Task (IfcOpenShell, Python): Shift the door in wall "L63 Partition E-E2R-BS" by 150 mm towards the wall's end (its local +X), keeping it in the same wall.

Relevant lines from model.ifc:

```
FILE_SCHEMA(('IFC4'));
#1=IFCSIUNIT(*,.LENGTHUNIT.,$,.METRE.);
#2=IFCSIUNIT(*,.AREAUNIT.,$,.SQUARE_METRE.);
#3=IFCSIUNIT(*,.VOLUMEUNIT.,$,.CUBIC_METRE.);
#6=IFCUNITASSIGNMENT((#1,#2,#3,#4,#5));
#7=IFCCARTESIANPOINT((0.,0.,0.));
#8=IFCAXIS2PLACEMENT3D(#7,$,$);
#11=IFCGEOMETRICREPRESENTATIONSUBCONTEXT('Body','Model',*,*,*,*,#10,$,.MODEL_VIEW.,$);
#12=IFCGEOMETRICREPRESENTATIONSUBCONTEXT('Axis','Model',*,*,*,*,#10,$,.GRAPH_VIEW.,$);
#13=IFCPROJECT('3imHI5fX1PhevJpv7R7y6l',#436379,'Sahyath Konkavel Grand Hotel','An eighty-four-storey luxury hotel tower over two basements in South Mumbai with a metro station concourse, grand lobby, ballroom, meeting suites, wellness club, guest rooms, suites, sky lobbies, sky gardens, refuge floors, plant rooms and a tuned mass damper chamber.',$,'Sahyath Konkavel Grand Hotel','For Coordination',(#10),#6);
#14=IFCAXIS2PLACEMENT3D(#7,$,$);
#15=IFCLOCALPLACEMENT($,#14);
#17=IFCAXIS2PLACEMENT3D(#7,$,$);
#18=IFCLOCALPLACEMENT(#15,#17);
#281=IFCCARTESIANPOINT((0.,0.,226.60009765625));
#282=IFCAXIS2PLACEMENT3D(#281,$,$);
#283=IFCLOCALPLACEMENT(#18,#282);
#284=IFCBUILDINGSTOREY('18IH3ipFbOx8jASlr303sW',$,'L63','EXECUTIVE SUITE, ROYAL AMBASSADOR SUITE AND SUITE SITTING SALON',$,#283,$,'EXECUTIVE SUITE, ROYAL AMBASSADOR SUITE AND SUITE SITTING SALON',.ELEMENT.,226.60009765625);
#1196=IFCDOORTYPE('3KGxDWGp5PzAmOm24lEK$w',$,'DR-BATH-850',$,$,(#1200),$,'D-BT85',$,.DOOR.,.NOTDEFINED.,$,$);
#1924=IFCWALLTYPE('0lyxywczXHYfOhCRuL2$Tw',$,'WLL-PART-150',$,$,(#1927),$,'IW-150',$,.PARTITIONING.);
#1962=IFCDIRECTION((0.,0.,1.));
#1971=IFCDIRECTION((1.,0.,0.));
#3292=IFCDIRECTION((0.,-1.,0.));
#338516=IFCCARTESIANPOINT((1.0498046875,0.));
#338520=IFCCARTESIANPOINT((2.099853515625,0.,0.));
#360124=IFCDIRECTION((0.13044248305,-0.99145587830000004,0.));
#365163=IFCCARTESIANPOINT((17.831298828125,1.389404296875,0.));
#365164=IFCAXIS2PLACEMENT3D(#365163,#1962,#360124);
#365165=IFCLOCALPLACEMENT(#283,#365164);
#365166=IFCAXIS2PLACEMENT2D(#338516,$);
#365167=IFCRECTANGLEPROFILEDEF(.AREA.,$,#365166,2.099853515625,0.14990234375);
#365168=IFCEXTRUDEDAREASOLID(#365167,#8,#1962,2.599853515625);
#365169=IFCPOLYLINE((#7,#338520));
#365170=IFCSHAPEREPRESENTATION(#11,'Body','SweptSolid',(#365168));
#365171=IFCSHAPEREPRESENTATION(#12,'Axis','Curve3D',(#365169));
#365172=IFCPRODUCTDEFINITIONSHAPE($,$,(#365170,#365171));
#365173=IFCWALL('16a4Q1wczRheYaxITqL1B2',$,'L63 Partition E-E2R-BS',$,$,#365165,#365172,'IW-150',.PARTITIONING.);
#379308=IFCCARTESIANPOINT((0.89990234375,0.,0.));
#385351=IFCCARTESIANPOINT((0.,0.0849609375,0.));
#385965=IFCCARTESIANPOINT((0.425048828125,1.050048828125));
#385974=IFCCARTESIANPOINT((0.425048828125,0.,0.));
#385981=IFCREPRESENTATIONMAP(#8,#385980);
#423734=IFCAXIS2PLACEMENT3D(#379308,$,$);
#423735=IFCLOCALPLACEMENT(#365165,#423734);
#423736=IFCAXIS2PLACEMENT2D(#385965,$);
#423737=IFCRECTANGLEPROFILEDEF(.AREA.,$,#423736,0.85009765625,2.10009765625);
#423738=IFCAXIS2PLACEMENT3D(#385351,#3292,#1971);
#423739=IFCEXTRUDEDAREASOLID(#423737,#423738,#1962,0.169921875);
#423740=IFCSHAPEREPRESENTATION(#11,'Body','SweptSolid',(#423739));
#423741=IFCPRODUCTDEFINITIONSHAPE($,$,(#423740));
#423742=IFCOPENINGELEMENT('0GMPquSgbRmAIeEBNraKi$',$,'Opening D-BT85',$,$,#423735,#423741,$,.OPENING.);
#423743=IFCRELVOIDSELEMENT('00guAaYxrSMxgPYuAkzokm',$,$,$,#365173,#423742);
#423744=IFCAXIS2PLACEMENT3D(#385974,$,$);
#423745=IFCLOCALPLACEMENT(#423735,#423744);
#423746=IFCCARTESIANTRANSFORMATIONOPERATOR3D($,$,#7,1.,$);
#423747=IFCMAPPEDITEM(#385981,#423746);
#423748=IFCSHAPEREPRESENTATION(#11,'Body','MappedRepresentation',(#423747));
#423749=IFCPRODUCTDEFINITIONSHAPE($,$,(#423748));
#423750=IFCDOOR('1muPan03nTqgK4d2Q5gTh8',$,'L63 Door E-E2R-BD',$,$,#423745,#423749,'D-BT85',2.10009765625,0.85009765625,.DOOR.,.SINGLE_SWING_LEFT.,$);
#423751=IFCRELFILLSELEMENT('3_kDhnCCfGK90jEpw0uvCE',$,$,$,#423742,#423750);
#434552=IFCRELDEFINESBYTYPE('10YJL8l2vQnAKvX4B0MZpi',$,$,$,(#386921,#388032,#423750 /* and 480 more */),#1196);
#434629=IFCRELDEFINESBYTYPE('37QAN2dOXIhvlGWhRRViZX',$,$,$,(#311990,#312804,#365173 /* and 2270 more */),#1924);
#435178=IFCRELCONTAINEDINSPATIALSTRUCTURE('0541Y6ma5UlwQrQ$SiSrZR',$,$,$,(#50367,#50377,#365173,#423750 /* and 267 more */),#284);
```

```python
import ifcopenshell
import ifcopenshell.api.geometry
import ifcopenshell.util.placement
import ifcopenshell.util.unit

model = ifcopenshell.open("model.ifc")
unit_scale = ifcopenshell.util.unit.calculate_unit_scale(model)

door = model.by_id(423750)
opening = door.FillsVoids[0].RelatingOpeningElement
wall = opening.VoidsElements[0].RelatingBuildingElement

wall_matrix = ifcopenshell.util.placement.get_local_placement(wall.ObjectPlacement)
shift = wall_matrix[:3, 0] * 0.15 / unit_scale
before = ifcopenshell.util.placement.get_local_placement(door.ObjectPlacement)[:3, 3].copy()

# The door is placed relative to its opening, so it follows when the opening moves.
matrix = ifcopenshell.util.placement.get_local_placement(opening.ObjectPlacement)
matrix[:3, 3] += shift
ifcopenshell.api.geometry.edit_object_placement(
    model, product=opening, matrix=matrix, is_si=False, should_transform_children=True
)

after = ifcopenshell.util.placement.get_local_placement(door.ObjectPlacement)[:3, 3]
print("door moved by", (after - before).round(3) + 0.0)

model.write("model-out.ifc")
```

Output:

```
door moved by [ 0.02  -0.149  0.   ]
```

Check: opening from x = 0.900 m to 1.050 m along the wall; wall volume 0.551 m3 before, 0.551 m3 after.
